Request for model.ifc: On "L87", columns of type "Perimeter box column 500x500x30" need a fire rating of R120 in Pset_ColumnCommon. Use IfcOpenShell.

First a look at what the model holds.

```python
import ifcopenshell
import ifcopenshell.util.element

model = ifcopenshell.open("model.ifc")
print(model.schema)
storey = next(s for s in model.by_type("IfcBuildingStorey") if s.Name == "L87")
columns = [e for e in ifcopenshell.util.element.get_decomposition(storey) if e.is_a("IfcColumn")]
seen = {}
for e in columns:
    element_type = ifcopenshell.util.element.get_type(e)
    key = (element_type.Name if element_type != e and element_type else None, ifcopenshell.util.element.get_pset(e, "Pset_ColumnCommon", "FireRating"))
    seen[key] = seen.get(key, 0) + 1
for (name, value), count in sorted(seen.items(), key=str):
    print(count, "x", name, "|", value)
```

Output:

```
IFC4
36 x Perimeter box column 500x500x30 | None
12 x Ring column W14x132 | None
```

```python
import ifcopenshell
import ifcopenshell.api.pset
import ifcopenshell.util.element

model = ifcopenshell.open("model.ifc")

storey = next(s for s in model.by_type("IfcBuildingStorey") if s.Name == "L87")
columns = [e for e in ifcopenshell.util.element.get_decomposition(storey) if e.is_a("IfcColumn")]

count = 0
for e in columns:
    element_type = ifcopenshell.util.element.get_type(e)
    if element_type in (None, e) or element_type.Name != "Perimeter box column 500x500x30":
        continue
    found = ifcopenshell.util.element.get_pset(e, "Pset_ColumnCommon", should_inherit=False)
    if found:
        pset = model.by_id(found["id"])
        if len(ifcopenshell.util.element.get_elements_by_pset(pset)) > 1:
            pset = ifcopenshell.api.pset.unshare_pset(model, products=[e], pset=pset)[0]
    else:
        pset = ifcopenshell.api.pset.add_pset(model, product=e, name="Pset_ColumnCommon")
    ifcopenshell.api.pset.edit_pset(model, pset=pset, properties={"FireRating": "R120"})
    count += 1

print(count, "columns updated")

model.write("model_v2.ifc")
```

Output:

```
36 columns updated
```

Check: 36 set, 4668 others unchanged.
